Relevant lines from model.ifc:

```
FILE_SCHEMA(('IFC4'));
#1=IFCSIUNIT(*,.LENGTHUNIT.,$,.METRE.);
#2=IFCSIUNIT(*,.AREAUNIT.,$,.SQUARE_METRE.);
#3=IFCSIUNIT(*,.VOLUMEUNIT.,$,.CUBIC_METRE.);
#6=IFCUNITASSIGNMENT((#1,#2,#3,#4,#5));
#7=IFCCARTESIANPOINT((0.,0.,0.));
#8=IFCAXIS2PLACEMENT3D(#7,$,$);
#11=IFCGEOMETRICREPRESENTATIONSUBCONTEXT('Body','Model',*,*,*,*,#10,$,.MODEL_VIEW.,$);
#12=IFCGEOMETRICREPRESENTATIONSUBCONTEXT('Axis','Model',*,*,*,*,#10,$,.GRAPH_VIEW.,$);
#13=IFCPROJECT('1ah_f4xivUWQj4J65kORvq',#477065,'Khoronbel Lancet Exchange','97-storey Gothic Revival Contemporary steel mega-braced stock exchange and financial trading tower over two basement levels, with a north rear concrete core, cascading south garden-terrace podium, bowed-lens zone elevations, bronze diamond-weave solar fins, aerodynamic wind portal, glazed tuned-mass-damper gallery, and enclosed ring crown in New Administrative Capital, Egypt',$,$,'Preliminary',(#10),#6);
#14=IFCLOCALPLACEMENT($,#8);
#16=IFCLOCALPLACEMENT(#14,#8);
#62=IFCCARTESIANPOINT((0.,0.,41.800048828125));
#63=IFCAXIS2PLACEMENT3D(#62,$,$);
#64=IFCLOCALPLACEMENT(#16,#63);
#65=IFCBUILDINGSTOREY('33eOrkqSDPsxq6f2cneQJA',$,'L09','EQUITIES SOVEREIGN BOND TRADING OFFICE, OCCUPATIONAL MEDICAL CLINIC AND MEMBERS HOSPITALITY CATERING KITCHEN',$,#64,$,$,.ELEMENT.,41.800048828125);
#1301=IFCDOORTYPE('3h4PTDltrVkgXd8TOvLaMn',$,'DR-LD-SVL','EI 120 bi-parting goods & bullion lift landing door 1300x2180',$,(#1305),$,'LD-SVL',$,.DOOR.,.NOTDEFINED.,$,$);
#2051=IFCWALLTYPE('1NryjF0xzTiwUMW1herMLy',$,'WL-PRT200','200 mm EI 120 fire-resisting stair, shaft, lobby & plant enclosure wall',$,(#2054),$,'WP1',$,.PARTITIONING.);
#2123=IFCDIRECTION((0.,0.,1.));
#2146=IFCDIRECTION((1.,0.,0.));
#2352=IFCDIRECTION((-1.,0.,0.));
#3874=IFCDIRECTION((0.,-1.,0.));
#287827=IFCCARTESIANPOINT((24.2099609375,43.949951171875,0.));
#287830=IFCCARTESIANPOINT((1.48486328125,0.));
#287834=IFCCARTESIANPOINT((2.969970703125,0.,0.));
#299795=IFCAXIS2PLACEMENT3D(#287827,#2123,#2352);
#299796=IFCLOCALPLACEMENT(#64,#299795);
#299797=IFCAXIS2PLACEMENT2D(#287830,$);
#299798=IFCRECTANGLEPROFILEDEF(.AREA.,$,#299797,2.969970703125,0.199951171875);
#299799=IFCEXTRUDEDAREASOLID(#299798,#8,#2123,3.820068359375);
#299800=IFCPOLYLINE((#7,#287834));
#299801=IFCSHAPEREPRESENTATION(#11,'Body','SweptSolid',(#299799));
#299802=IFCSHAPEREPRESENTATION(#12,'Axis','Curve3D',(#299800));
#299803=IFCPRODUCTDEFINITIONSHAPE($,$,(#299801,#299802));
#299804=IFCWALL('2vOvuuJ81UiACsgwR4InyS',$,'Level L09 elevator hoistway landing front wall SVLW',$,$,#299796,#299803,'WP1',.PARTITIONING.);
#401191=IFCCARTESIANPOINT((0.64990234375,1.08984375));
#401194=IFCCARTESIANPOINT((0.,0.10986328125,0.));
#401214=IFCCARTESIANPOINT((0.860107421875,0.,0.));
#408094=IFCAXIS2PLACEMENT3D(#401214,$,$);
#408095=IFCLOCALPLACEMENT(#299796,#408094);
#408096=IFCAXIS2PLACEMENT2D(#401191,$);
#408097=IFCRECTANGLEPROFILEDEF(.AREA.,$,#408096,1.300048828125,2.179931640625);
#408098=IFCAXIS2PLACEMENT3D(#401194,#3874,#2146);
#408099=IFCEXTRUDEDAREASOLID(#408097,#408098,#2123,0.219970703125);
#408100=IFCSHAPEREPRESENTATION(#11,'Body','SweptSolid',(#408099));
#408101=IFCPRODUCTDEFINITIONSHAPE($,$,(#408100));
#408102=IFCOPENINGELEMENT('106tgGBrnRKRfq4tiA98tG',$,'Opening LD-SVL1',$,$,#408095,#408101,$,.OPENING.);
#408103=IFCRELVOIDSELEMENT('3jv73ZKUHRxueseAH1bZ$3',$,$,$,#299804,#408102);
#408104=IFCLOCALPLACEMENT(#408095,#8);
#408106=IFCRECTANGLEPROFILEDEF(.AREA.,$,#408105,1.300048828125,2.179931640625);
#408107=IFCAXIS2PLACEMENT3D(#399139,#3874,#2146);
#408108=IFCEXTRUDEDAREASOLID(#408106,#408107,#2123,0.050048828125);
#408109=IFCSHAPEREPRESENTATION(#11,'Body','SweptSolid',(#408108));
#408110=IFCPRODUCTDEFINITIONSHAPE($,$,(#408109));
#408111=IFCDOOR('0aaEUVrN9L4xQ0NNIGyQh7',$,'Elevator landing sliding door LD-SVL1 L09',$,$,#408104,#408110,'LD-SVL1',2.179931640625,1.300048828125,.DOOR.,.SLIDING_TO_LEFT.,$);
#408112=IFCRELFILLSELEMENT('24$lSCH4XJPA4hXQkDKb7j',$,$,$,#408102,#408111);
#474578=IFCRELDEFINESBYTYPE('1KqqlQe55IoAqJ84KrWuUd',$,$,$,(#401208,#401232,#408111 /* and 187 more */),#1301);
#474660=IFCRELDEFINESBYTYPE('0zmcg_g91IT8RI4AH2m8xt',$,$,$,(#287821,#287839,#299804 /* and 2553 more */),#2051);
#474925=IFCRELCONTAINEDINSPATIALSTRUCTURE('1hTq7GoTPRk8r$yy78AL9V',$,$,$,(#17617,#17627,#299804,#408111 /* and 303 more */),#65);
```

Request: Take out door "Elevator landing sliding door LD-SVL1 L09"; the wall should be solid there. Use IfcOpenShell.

```python
import ifcopenshell
import ifcopenshell.api.feature
import ifcopenshell.api.root
import ifcopenshell.geom
import ifcopenshell.util.shape

model = ifcopenshell.open("model.ifc")
settings = ifcopenshell.geom.settings()


def volume(element):
    """Net volume in cubic metres, openings subtracted."""
    shape = ifcopenshell.geom.create_shape(settings, element)
    return ifcopenshell.util.shape.get_volume(shape.geometry)


door = model.by_id(408111)
opening = door.FillsVoids[0].RelatingOpeningElement
wall = opening.VoidsElements[0].RelatingBuildingElement
before = volume(wall)

ifcopenshell.api.root.remove_product(model, product=door)
ifcopenshell.api.feature.remove_feature(model, feature=opening)

after = volume(wall)

print(f"wall volume {before:.3f} -> {after:.3f} m3")

model.write("model-out.ifc")
```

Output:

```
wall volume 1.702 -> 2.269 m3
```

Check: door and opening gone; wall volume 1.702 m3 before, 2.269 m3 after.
